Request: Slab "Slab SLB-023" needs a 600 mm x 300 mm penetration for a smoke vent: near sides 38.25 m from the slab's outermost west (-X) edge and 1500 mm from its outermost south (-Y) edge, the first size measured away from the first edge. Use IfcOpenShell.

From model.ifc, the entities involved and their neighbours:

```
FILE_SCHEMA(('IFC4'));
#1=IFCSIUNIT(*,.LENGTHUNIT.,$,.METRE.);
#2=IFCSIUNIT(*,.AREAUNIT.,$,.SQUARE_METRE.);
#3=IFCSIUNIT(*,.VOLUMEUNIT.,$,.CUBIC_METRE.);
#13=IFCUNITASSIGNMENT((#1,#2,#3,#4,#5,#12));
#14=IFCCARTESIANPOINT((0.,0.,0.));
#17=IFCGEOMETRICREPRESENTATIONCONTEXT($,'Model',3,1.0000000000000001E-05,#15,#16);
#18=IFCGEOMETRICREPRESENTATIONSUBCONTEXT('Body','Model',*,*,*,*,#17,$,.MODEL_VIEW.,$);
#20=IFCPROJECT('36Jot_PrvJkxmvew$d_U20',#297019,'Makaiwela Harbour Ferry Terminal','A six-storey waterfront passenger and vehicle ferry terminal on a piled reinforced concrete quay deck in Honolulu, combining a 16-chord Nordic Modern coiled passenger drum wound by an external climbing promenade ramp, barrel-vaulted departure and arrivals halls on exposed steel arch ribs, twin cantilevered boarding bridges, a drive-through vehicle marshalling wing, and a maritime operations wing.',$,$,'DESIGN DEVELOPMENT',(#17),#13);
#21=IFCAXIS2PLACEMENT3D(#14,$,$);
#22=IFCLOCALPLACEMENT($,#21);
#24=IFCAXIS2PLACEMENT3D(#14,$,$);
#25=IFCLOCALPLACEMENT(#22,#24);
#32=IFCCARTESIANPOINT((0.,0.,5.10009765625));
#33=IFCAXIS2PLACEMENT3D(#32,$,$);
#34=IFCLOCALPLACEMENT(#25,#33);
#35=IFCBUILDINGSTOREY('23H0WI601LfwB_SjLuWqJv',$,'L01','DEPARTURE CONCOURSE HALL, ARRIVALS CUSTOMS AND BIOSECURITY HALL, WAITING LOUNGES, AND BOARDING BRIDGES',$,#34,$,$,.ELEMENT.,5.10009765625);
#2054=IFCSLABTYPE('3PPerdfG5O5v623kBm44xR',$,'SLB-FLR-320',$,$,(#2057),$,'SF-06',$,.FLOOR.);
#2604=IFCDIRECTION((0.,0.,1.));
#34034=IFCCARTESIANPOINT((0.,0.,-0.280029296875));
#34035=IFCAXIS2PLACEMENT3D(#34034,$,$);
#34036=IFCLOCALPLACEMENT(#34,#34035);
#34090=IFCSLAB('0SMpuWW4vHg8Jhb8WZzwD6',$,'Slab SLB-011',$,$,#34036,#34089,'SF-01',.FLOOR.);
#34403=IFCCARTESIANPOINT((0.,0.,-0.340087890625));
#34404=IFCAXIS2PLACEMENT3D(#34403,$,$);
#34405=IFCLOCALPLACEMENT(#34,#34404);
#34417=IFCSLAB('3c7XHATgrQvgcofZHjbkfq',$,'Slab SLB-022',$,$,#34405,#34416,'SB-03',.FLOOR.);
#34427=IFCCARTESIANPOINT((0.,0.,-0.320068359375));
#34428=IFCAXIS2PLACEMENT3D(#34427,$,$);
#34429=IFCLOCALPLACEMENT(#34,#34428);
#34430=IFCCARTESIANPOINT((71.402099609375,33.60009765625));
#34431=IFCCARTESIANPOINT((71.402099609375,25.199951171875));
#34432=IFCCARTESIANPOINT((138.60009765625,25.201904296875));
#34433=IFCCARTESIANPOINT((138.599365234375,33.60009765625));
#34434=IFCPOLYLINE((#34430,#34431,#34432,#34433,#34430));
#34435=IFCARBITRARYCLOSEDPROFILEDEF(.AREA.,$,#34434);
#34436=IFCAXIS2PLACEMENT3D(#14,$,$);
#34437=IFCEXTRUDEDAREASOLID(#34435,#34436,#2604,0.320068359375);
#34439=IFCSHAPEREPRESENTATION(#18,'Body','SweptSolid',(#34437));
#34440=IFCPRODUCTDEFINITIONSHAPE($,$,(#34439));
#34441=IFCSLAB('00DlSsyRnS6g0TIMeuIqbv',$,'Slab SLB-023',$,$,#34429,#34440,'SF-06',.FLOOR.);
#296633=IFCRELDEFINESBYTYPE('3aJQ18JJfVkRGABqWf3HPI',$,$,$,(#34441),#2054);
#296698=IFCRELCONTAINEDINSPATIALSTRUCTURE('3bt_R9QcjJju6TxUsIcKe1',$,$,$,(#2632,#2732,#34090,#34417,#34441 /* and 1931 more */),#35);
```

```python
import numpy as np
import ifcopenshell
import ifcopenshell.api.feature
import ifcopenshell.api.geometry
import ifcopenshell.api.root
import ifcopenshell.geom
import ifcopenshell.util.placement
import ifcopenshell.util.representation
import ifcopenshell.util.shape
import ifcopenshell.util.unit

model = ifcopenshell.open("model.ifc")
unit_scale = ifcopenshell.util.unit.calculate_unit_scale(model)
settings = ifcopenshell.geom.settings()


def volume(element):
    """Net volume in cubic metres, openings subtracted."""
    shape = ifcopenshell.geom.create_shape(settings, element)
    return ifcopenshell.util.shape.get_volume(shape.geometry)


slab = model.by_guid("00DlSsyRnS6g0TIMeuIqbv")
before = volume(slab)

# Extent in the slab's own axes, in metres. The edges named are its -X and -Y sides.
slab_shape = ifcopenshell.geom.create_shape(settings, slab)
vertices = ifcopenshell.util.shape.get_vertices(slab_shape.geometry)
x_min, y_min, bottom = vertices.min(axis=0)
top = vertices[:, 2].max()

opening = ifcopenshell.api.root.create_entity(model, ifc_class="IfcOpeningElement", name="Smoke vent opening", predefined_type="OPENING")
context = ifcopenshell.util.representation.get_context(model, "Model", "Body", "MODEL_VIEW")
width, depth = 0.6, 0.3
outline = [(0.0, 0.0), (width, 0.0), (width, depth), (0.0, depth), (0.0, 0.0)]
# Overshoot both faces by 50 mm so the cut is clean.
shape = ifcopenshell.api.geometry.add_slab_representation(
    model, context=context, depth=top - bottom + 0.1, polyline=outline
)
ifcopenshell.api.geometry.assign_representation(model, product=opening, representation=shape)

matrix = ifcopenshell.util.placement.get_local_placement(slab.ObjectPlacement)
matrix[:, 3] = matrix @ np.append(np.array([x_min + 38.25, y_min + 1.5, bottom - 0.05]) / unit_scale, 1.0)
ifcopenshell.api.geometry.edit_object_placement(model, product=opening, matrix=matrix, is_si=False)
ifcopenshell.api.feature.add_feature(model, feature=opening, element=slab)

after = volume(slab)

print(f"slab volume {before:.3f} -> {after:.3f} m3")

model.write("model_v2.ifc")
```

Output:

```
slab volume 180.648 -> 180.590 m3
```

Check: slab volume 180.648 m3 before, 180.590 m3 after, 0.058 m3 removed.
